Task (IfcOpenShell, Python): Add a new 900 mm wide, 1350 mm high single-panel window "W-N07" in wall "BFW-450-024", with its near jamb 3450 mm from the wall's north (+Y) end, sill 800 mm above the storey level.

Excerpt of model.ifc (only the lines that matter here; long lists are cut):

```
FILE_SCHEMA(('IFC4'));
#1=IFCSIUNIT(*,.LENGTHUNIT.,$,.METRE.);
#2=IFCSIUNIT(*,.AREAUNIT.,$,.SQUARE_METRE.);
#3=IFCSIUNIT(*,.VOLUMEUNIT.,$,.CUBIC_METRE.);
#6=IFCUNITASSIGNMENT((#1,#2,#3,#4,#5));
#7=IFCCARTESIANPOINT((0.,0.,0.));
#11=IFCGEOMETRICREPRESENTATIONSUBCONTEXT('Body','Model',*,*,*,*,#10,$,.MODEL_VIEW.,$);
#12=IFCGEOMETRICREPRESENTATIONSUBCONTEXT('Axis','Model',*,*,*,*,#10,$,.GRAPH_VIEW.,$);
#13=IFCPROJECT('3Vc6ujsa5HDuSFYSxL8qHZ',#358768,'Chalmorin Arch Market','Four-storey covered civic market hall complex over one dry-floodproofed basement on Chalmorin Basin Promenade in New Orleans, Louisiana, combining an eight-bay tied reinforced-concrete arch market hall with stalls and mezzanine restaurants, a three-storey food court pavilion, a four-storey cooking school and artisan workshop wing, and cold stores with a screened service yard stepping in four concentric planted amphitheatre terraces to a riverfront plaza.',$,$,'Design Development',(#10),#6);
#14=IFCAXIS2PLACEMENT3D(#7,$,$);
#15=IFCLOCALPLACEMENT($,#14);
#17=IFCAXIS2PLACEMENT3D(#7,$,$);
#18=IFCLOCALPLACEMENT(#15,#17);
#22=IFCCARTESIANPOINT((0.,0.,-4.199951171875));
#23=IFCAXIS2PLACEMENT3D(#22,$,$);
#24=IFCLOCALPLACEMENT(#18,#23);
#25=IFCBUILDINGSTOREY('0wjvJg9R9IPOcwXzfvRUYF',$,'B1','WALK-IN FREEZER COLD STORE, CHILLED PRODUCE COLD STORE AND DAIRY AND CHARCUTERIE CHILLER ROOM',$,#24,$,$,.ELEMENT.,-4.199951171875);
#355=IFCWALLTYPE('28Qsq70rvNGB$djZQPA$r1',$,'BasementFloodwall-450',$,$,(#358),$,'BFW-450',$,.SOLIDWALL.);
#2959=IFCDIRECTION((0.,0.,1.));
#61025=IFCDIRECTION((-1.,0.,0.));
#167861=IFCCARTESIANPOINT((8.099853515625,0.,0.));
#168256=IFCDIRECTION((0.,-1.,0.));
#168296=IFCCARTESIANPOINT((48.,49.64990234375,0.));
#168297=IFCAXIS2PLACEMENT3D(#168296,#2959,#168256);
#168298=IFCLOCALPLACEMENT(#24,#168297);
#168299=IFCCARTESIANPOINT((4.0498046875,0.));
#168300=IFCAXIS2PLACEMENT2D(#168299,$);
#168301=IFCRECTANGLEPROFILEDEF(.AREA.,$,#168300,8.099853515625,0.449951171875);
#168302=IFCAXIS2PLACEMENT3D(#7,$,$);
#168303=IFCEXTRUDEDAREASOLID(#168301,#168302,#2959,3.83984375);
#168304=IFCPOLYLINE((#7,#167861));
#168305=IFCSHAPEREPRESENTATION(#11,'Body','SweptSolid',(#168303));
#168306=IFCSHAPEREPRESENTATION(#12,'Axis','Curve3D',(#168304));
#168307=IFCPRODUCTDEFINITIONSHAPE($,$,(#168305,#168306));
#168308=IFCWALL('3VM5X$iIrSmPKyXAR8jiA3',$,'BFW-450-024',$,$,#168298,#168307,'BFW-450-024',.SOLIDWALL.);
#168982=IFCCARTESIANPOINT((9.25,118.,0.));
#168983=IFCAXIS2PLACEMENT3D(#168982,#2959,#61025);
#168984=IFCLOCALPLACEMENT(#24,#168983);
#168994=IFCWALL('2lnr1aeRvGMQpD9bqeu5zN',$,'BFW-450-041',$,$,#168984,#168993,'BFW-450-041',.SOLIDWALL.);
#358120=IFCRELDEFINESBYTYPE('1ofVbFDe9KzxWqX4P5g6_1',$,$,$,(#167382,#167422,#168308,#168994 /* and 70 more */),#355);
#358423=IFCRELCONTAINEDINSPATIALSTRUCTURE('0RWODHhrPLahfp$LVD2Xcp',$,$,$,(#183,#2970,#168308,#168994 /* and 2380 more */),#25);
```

```python
import numpy as np
import ifcopenshell
import ifcopenshell.api.feature
import ifcopenshell.api.geometry
import ifcopenshell.api.root
import ifcopenshell.api.spatial
import ifcopenshell.geom
import ifcopenshell.util.element
import ifcopenshell.util.placement
import ifcopenshell.util.representation
import ifcopenshell.util.shape
import ifcopenshell.util.unit

model = ifcopenshell.open("model.ifc")
unit_scale = ifcopenshell.util.unit.calculate_unit_scale(model)
settings = ifcopenshell.geom.settings()


def volume(element):
    """Net volume in cubic metres, openings subtracted."""
    shape = ifcopenshell.geom.create_shape(settings, element)
    return ifcopenshell.util.shape.get_volume(shape.geometry)


wall = model.by_id(168308)
storey = ifcopenshell.util.element.get_container(wall, ifc_class="IfcBuildingStorey")
context = ifcopenshell.util.representation.get_context(model, "Model", "Body", "MODEL_VIEW")
before = volume(wall)

width, height, from_end, sill = 0.9, 1.35, 3.45, 0.8  # metres

# The wall runs along its own X axis, and the end named is its -X end.
wall_shape = ifcopenshell.geom.create_shape(settings, wall)
x, y, z = ifcopenshell.util.shape.get_vertices(wall_shape.geometry).T
start = x.min() + from_end
face, thickness = float(y.min()), float(y.max() - y.min())
wall_matrix = ifcopenshell.util.placement.get_local_placement(wall.ObjectPlacement)
level = ifcopenshell.util.placement.get_local_placement(storey.ObjectPlacement)[2, 3]


def in_wall(x, y):
    """Placement at x, y metres in the wall's axes, at sill height."""
    matrix = wall_matrix.copy()
    matrix[:, 3] = wall_matrix @ np.array([x / unit_scale, y / unit_scale, 0.0, 1.0])
    matrix[2, 3] = level + sill / unit_scale
    return matrix


# Opening: a box that overshoots both wall faces by 50 mm.
opening = ifcopenshell.api.root.create_entity(model, ifc_class="IfcOpeningElement", predefined_type="OPENING")
box = ifcopenshell.api.geometry.add_wall_representation(
    model, context=context, length=width, height=height, thickness=thickness + 0.1
)
ifcopenshell.api.geometry.assign_representation(model, product=opening, representation=box)
ifcopenshell.api.geometry.edit_object_placement(model, product=opening, matrix=in_wall(start, face - 0.05), is_si=False)
ifcopenshell.api.feature.add_feature(model, feature=opening, element=wall)

window = ifcopenshell.api.root.create_entity(model, ifc_class="IfcWindow", name="W-N07", predefined_type="WINDOW")
window.OverallWidth, window.OverallHeight = width / unit_scale, height / unit_scale
window.PartitioningType = "SINGLE_PANEL"
body = ifcopenshell.api.geometry.add_window_representation(
    model,
    context=context,
    overall_width=window.OverallWidth,
    overall_height=window.OverallHeight,
    partition_type="SINGLE_PANEL",
)
ifcopenshell.api.geometry.assign_representation(model, product=window, representation=body)
ifcopenshell.api.spatial.assign_container(model, products=[window], relating_structure=storey)
ifcopenshell.api.feature.add_filling(model, opening=opening, element=window)

# Centre the window in the wall's thickness.
ifcopenshell.api.geometry.edit_object_placement(model, product=window, matrix=in_wall(start, face), is_si=False)
window_shape = ifcopenshell.geom.create_shape(settings, window)
depth = ifcopenshell.util.shape.get_vertices(window_shape.geometry)[:, 1]
offset = face + thickness / 2 - (depth.min() + depth.max()) / 2
ifcopenshell.api.geometry.edit_object_placement(model, product=window, matrix=in_wall(start, offset), is_si=False)

after = volume(wall)

print(f"wall volume {before:.3f} -> {after:.3f} m3")

model.write("model-out.ifc")
```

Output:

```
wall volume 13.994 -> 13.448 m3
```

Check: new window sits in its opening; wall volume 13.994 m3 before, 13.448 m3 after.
